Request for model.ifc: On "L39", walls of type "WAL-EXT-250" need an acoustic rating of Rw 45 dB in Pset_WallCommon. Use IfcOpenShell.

First a look at what the model holds.

```python
import ifcopenshell
import ifcopenshell.util.element

model = ifcopenshell.open("model.ifc")
print(model.schema)
storey = next(s for s in model.by_type("IfcBuildingStorey") if s.Name == "L39")
walls = [e for e in ifcopenshell.util.element.get_decomposition(storey) if e.is_a("IfcWall")]
seen = {}
for e in walls:
    element_type = ifcopenshell.util.element.get_type(e)
    key = (element_type.Name if element_type != e and element_type else None, ifcopenshell.util.element.get_pset(e, "Pset_WallCommon", "AcousticRating"))
    seen[key] = seen.get(key, 0) + 1
for (name, value), count in sorted(seen.items(), key=str):
    print(count, "x", name, "|", value)
```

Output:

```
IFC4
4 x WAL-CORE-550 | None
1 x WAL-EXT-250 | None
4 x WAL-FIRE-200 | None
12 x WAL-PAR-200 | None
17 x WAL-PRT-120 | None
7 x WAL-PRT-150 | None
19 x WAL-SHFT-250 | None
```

```python
import ifcopenshell
import ifcopenshell.api.pset
import ifcopenshell.util.element

model = ifcopenshell.open("model.ifc")

storey = next(s for s in model.by_type("IfcBuildingStorey") if s.Name == "L39")
walls = [e for e in ifcopenshell.util.element.get_decomposition(storey) if e.is_a("IfcWall")]

count = 0
for e in walls:
    element_type = ifcopenshell.util.element.get_type(e)
    if element_type in (None, e) or element_type.Name != "WAL-EXT-250":
        continue
    # add_pset returns the element's existing set when there is one.
    pset = ifcopenshell.api.pset.add_pset(model, product=e, name="Pset_WallCommon")
    ifcopenshell.api.pset.edit_pset(model, pset=pset, properties={"AcousticRating": "Rw 45 dB"})
    count += 1

print(count, "walls updated")

model.write("model_updated.ifc")
```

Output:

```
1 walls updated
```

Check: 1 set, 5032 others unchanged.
